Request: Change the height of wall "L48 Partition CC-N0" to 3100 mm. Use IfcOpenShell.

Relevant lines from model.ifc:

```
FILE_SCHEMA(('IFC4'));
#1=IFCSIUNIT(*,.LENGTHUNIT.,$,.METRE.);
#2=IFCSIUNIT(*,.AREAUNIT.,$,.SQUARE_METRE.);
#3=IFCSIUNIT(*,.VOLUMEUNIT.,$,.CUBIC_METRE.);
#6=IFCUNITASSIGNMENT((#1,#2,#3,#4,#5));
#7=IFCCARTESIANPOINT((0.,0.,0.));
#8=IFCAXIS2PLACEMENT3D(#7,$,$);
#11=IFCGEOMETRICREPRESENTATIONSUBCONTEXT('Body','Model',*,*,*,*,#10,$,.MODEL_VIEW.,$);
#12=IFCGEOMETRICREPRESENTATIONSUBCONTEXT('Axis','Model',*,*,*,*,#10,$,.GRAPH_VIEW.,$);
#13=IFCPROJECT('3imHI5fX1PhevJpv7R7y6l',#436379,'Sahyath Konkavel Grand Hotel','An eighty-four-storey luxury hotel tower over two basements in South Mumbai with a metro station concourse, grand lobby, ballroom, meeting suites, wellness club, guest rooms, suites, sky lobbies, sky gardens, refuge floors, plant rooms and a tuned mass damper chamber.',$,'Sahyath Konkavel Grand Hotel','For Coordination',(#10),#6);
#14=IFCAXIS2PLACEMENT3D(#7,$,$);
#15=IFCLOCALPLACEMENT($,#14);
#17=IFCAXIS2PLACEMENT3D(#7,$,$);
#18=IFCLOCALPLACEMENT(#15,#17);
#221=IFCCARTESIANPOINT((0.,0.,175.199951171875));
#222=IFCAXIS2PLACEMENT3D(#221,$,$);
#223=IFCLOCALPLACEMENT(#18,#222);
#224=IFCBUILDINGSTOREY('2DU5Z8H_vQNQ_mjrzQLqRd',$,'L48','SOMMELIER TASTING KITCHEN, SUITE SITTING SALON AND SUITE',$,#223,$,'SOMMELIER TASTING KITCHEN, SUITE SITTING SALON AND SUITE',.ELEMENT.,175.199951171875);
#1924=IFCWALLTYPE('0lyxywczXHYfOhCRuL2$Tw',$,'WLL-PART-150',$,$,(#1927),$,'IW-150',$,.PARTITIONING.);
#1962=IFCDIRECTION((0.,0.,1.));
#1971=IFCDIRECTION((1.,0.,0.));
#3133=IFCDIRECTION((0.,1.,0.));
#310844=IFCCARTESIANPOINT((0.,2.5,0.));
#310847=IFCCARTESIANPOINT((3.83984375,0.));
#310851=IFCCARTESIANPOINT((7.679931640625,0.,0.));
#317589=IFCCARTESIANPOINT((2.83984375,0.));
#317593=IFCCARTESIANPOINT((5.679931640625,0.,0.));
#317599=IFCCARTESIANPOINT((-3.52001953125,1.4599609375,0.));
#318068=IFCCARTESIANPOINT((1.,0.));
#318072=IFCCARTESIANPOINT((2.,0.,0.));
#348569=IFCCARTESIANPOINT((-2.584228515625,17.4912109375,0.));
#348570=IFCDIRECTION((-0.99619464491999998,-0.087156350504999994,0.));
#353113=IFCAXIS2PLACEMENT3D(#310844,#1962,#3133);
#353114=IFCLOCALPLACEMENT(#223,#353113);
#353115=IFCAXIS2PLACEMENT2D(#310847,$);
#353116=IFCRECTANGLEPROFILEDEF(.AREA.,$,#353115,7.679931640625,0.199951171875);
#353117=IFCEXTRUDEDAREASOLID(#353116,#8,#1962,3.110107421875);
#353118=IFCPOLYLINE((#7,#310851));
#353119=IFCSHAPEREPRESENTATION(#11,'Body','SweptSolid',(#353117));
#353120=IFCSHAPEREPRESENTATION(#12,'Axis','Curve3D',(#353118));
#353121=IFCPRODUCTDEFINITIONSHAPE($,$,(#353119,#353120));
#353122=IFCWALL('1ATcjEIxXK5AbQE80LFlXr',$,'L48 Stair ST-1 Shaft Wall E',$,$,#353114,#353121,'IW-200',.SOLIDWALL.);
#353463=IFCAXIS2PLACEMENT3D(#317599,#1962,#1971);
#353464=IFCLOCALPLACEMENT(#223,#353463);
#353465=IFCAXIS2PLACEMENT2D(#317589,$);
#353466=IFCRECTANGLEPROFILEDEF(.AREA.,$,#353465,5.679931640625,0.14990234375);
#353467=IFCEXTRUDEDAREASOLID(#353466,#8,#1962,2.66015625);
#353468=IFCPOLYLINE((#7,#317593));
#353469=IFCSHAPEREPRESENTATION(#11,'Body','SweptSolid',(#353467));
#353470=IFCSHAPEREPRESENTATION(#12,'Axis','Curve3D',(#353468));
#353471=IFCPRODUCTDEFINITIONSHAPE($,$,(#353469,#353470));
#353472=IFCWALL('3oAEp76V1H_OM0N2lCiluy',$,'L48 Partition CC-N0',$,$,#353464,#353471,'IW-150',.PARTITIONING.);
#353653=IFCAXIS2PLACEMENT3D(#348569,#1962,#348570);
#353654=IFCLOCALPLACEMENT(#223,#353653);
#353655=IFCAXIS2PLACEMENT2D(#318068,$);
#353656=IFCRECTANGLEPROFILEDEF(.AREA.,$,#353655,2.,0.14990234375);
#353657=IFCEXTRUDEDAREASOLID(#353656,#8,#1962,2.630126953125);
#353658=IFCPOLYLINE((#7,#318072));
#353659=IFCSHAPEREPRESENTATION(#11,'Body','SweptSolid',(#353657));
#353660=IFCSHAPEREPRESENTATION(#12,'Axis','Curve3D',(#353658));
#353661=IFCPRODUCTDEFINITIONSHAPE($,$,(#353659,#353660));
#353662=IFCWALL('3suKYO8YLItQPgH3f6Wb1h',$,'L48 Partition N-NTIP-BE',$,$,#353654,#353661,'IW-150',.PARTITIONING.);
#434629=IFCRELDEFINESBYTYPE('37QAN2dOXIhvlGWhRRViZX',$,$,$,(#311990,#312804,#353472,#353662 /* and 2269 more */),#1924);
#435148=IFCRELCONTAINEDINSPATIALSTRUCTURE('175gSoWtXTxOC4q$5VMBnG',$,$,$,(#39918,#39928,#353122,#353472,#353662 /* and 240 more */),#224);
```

```python
import ifcopenshell
import ifcopenshell.geom
import ifcopenshell.util.representation
import ifcopenshell.util.shape

model = ifcopenshell.open("model.ifc")
settings = ifcopenshell.geom.settings()


def volume(element):
    """Net volume in cubic metres, openings subtracted."""
    shape = ifcopenshell.geom.create_shape(settings, element)
    return ifcopenshell.util.shape.get_volume(shape.geometry)


wall = model.by_id(353472)
before = volume(wall)

body = ifcopenshell.util.representation.get_representation(wall, "Model", "Body")
solid = body.Items[0]
old_height = solid.Depth
solid.Depth = 3.1
after = volume(wall)

print(f"height {old_height:g} -> {solid.Depth:g}, volume {before:.3f} -> {after:.3f} m3")

model.write("model_rev.ifc")
```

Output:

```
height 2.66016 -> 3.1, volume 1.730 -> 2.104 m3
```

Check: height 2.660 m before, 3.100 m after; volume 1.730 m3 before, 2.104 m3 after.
